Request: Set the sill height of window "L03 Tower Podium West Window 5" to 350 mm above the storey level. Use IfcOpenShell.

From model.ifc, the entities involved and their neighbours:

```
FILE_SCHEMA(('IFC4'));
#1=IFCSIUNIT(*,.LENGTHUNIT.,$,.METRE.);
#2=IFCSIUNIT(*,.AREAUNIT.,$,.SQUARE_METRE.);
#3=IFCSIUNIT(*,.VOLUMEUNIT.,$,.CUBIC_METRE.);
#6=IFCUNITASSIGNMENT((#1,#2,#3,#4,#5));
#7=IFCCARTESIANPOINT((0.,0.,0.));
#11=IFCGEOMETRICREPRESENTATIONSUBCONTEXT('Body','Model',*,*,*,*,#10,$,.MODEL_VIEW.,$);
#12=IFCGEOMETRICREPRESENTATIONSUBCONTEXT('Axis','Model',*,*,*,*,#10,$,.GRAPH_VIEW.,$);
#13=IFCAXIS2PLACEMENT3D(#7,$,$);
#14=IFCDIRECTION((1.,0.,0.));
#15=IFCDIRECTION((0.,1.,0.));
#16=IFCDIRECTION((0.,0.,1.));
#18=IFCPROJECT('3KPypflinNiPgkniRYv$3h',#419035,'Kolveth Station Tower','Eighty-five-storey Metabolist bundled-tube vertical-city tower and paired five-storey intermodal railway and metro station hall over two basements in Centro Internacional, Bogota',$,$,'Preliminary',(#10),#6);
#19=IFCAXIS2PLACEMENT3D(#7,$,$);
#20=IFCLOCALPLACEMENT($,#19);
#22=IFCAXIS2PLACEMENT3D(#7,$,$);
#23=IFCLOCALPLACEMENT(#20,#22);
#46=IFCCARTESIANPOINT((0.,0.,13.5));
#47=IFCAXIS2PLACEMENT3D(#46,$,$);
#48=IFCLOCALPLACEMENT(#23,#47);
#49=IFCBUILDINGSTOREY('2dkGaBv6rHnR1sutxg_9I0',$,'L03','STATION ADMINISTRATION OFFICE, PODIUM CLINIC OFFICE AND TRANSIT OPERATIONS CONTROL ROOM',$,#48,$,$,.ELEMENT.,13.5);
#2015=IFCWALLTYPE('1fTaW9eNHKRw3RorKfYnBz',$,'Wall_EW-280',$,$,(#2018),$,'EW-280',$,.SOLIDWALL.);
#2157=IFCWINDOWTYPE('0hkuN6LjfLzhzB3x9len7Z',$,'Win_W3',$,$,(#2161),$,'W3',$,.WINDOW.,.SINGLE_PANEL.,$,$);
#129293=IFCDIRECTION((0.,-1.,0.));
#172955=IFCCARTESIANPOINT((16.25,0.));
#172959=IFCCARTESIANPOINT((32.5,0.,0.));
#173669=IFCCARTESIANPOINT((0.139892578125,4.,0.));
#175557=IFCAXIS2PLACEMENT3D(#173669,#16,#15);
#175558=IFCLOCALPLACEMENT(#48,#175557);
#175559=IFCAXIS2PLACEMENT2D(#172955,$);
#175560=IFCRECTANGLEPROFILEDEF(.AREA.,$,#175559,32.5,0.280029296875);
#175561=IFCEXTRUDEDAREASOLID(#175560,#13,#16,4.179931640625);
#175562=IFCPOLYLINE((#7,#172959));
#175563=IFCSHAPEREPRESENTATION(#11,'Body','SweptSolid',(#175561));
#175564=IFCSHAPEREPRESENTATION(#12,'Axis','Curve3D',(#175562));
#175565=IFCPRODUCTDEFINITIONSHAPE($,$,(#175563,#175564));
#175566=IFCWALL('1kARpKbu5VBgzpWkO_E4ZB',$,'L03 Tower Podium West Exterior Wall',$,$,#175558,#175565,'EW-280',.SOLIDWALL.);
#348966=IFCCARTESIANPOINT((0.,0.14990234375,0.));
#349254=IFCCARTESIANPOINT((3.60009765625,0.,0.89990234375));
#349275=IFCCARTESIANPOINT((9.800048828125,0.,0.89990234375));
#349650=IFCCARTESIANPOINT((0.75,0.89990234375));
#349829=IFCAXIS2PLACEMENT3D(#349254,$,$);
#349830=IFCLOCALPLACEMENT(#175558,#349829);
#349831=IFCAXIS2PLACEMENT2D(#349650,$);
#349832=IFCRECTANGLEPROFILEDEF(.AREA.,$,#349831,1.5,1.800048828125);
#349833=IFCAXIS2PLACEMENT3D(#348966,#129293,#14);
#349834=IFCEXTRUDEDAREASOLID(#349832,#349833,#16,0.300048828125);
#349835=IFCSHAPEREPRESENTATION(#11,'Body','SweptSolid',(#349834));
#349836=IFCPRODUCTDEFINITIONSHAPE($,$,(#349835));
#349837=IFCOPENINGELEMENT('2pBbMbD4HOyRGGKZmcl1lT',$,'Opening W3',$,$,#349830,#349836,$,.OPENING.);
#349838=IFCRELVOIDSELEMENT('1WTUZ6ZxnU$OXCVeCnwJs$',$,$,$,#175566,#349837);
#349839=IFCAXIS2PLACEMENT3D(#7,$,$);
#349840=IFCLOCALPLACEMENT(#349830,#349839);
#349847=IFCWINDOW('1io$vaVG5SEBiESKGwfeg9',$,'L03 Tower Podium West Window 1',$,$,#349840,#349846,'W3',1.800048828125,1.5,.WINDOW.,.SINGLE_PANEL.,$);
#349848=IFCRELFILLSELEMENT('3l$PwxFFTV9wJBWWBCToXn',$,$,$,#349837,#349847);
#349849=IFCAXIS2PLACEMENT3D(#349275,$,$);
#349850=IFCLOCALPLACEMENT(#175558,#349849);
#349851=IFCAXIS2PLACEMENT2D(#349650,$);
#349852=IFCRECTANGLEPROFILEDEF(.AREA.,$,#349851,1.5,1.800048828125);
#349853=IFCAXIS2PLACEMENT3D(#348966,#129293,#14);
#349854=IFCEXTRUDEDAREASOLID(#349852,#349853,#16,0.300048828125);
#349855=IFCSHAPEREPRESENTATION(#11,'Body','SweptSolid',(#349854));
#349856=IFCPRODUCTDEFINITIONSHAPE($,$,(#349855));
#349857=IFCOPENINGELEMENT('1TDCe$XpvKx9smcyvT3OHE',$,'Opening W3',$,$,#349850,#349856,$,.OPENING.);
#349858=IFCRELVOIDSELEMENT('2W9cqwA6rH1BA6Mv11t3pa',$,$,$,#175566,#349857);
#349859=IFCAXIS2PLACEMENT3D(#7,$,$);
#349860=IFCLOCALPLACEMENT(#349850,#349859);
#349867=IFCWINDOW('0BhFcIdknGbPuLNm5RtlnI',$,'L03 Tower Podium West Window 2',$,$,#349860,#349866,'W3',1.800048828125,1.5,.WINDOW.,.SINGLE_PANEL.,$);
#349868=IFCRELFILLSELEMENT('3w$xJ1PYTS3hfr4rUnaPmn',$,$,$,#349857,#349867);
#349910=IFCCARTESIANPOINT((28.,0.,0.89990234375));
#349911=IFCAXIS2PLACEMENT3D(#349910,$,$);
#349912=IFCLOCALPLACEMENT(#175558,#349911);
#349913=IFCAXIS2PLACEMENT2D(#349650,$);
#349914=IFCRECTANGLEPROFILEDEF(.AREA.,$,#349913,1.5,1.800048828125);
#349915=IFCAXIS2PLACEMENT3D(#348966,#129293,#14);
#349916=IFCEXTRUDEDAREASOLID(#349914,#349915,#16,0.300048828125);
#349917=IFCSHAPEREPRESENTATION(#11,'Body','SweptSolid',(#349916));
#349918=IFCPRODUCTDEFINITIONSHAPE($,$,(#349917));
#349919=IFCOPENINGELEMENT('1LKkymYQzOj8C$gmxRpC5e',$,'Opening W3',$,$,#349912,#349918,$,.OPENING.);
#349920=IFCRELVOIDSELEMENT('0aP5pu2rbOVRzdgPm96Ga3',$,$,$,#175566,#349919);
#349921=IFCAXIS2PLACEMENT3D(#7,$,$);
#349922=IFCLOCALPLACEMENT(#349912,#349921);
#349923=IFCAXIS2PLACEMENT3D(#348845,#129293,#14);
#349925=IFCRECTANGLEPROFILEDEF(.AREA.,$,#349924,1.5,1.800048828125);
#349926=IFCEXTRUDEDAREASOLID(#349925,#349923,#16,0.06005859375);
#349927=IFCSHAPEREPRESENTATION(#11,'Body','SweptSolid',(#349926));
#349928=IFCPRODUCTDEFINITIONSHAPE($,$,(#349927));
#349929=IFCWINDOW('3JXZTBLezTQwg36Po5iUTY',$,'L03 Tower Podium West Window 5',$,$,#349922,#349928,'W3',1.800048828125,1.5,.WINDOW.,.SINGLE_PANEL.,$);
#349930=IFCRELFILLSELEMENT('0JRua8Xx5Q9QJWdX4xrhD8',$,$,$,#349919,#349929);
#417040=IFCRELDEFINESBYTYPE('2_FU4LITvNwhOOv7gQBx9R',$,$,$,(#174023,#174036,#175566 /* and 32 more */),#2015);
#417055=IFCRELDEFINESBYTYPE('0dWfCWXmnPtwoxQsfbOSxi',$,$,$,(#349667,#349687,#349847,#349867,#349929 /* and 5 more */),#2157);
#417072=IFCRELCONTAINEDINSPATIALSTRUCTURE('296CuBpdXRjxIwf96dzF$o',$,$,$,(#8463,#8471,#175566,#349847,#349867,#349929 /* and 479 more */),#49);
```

```python
import numpy as np
import ifcopenshell
import ifcopenshell.api.geometry
import ifcopenshell.geom
import ifcopenshell.util.element
import ifcopenshell.util.placement
import ifcopenshell.util.shape
import ifcopenshell.util.unit

model = ifcopenshell.open("model.ifc")
unit_scale = ifcopenshell.util.unit.calculate_unit_scale(model)

window = model.by_id(349929)
opening = window.FillsVoids[0].RelatingOpeningElement
storey = ifcopenshell.util.element.get_container(window, ifc_class="IfcBuildingStorey")
level = ifcopenshell.util.placement.get_local_placement(storey.ObjectPlacement)[2, 3]

# The opening's origin need not be at the sill, so measure its lowest point.
shape = ifcopenshell.geom.create_shape(ifcopenshell.geom.settings(), opening)
bottom = ifcopenshell.util.shape.get_shape_bottom_elevation(shape, shape.geometry) / unit_scale
dz = level + 0.35 / unit_scale - bottom

shift = np.array([0.0, 0.0, dz])
# The window is placed relative to its opening, so it follows when the opening moves.
matrix = ifcopenshell.util.placement.get_local_placement(opening.ObjectPlacement)
matrix[:3, 3] += shift
ifcopenshell.api.geometry.edit_object_placement(
    model, product=opening, matrix=matrix, is_si=False, should_transform_children=True
)

print(f"moved by {dz * unit_scale:+.3f} m")

model.write("model_updated.ifc")
```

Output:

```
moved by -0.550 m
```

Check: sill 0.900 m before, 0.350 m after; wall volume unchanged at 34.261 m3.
